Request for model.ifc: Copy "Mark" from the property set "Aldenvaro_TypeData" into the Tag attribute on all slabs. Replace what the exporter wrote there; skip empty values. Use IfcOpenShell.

First a look at what the model holds.

```python
import ifcopenshell
import ifcopenshell.util.element

model = ifcopenshell.open("model.ifc")
print(model.schema)
slabs = model.by_type("IfcSlab")
print(len(slabs), "slabs")
for e in slabs[:8]:
    source = ifcopenshell.util.element.get_pset(e, "Aldenvaro_TypeData", "Mark")
    target = e.Tag
    print(e.id(), repr(source), repr(target), sep=" | ")
```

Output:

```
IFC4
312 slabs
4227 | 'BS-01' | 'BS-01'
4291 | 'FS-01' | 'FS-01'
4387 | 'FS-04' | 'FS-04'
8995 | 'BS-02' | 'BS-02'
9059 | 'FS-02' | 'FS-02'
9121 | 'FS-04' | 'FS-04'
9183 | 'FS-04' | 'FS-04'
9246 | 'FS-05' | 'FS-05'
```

```python
import ifcopenshell
import ifcopenshell.util.element

model = ifcopenshell.open("model.ifc")

count = 0
for e in model.by_type("IfcSlab"):
    value = ifcopenshell.util.element.get_pset(e, "Aldenvaro_TypeData", "Mark")
    current = e.Tag
    if not value or not value.strip() or current == value:
        continue
    e.Tag = value
    count += 1

print(count, "slabs updated")

model.write("model_v2.ifc")
```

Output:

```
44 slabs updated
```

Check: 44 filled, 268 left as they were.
